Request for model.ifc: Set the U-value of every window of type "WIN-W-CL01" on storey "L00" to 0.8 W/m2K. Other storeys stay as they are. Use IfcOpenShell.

First a look at what the model holds.

```python
import ifcopenshell
import ifcopenshell.util.element

model = ifcopenshell.open("model.ifc")
print(model.schema)
storey = next(s for s in model.by_type("IfcBuildingStorey") if s.Name == "L00")
windows = [e for e in ifcopenshell.util.element.get_decomposition(storey) if e.is_a("IfcWindow")]
seen = {}
for e in windows:
    element_type = ifcopenshell.util.element.get_type(e)
    key = (element_type.Name if element_type != e and element_type else None, ifcopenshell.util.element.get_pset(e, "Pset_WindowCommon", "ThermalTransmittance"))
    seen[key] = seen.get(key, 0) + 1
for (name, value), count in sorted(seen.items(), key=str):
    print(count, "x", name, "|", value)
```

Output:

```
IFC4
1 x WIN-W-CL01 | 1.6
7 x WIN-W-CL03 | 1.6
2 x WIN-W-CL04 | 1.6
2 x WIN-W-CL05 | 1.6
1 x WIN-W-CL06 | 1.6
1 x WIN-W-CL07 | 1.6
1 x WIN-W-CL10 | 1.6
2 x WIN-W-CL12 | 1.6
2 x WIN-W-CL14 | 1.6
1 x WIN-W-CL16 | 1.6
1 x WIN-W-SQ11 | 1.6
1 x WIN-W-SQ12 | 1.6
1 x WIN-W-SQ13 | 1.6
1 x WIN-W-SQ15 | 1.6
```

```python
import ifcopenshell
import ifcopenshell.api.pset
import ifcopenshell.util.element

model = ifcopenshell.open("model.ifc")

storey = next(s for s in model.by_type("IfcBuildingStorey") if s.Name == "L00")
windows = [e for e in ifcopenshell.util.element.get_decomposition(storey) if e.is_a("IfcWindow")]

count = 0
for e in windows:
    element_type = ifcopenshell.util.element.get_type(e)
    if element_type in (None, e) or element_type.Name != "WIN-W-CL01":
        continue
    # add_pset returns the element's existing set when there is one.
    pset = ifcopenshell.api.pset.add_pset(model, product=e, name="Pset_WindowCommon")
    ifcopenshell.api.pset.edit_pset(model, pset=pset, properties={"ThermalTransmittance": 0.8})
    count += 1

print(count, "windows updated")

model.write("model_updated.ifc")
```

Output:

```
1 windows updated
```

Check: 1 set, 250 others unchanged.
